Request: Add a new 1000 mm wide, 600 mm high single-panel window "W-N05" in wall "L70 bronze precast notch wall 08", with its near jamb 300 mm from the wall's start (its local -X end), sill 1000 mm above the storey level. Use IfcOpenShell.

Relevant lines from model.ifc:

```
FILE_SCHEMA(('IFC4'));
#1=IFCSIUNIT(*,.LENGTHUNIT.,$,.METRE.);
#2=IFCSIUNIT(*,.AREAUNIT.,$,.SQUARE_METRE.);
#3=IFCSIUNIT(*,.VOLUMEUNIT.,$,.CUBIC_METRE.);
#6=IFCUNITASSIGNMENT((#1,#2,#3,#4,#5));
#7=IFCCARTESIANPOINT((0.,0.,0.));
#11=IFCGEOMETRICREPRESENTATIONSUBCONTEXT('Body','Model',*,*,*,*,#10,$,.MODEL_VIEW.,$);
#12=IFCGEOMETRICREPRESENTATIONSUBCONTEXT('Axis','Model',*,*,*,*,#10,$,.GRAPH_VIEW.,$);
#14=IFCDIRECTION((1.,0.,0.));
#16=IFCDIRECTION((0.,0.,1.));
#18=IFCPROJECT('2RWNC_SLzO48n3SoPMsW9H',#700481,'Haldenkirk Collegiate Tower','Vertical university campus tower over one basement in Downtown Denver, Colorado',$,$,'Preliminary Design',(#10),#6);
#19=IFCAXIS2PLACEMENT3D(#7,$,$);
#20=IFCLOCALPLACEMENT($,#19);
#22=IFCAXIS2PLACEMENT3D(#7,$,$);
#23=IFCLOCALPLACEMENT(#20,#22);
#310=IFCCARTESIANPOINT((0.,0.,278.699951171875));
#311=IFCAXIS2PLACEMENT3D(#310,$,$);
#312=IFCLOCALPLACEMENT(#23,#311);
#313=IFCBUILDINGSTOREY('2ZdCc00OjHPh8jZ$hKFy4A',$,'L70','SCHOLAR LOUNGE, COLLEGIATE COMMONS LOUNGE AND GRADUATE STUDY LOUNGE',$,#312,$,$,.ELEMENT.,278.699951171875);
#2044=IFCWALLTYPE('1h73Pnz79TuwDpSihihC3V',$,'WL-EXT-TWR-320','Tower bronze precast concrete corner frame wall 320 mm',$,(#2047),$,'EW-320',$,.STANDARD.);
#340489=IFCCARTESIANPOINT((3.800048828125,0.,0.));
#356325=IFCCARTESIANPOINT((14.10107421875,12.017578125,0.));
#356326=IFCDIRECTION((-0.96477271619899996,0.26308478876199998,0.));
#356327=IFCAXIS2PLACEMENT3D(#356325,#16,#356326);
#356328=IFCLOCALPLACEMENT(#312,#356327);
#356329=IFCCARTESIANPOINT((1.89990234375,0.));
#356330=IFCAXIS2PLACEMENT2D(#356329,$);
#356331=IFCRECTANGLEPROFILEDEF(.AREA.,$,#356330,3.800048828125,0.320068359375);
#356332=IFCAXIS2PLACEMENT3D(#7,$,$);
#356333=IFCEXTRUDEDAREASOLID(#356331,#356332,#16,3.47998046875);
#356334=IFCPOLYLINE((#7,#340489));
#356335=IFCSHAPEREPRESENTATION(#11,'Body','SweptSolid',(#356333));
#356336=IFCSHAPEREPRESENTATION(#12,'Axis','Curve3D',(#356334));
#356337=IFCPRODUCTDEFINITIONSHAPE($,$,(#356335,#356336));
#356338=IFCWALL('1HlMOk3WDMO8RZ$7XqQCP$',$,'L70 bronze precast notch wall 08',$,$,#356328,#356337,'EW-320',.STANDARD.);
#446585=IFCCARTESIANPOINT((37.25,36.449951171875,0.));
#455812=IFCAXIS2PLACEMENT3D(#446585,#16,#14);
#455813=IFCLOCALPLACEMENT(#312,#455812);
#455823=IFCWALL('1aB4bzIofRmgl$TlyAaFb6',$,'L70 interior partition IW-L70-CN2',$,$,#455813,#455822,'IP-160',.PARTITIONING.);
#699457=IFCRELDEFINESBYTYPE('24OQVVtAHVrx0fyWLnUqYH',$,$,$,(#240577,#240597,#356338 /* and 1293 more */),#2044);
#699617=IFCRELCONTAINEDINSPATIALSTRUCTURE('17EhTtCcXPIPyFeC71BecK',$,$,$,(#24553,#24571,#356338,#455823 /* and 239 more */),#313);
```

```python
import numpy as np
import ifcopenshell
import ifcopenshell.api.feature
import ifcopenshell.api.geometry
import ifcopenshell.api.root
import ifcopenshell.api.spatial
import ifcopenshell.geom
import ifcopenshell.util.element
import ifcopenshell.util.placement
import ifcopenshell.util.representation
import ifcopenshell.util.shape
import ifcopenshell.util.unit

model = ifcopenshell.open("model.ifc")
unit_scale = ifcopenshell.util.unit.calculate_unit_scale(model)
settings = ifcopenshell.geom.settings()


def volume(element):
    """Net volume in cubic metres, openings subtracted."""
    shape = ifcopenshell.geom.create_shape(settings, element)
    return ifcopenshell.util.shape.get_volume(shape.geometry)


wall = model.by_guid("1HlMOk3WDMO8RZ$7XqQCP$")
storey = ifcopenshell.util.element.get_container(wall, ifc_class="IfcBuildingStorey")
context = ifcopenshell.util.representation.get_context(model, "Model", "Body", "MODEL_VIEW")
before = volume(wall)

width, height, from_end, sill = 1, 0.6, 0.3, 1  # metres

# The wall runs along its own X axis, and the end named is its -X end.
wall_shape = ifcopenshell.geom.create_shape(settings, wall)
x, y, z = ifcopenshell.util.shape.get_vertices(wall_shape.geometry).T
start = x.min() + from_end
face, thickness = float(y.min()), float(y.max() - y.min())
wall_matrix = ifcopenshell.util.placement.get_local_placement(wall.ObjectPlacement)
level = ifcopenshell.util.placement.get_local_placement(storey.ObjectPlacement)[2, 3]


def in_wall(x, y):
    """Placement at x, y metres in the wall's axes, at sill height."""
    matrix = wall_matrix.copy()
    matrix[:, 3] = wall_matrix @ np.array([x / unit_scale, y / unit_scale, 0.0, 1.0])
    matrix[2, 3] = level + sill / unit_scale
    return matrix


# Opening: a box that overshoots both wall faces by 50 mm.
opening = ifcopenshell.api.root.create_entity(model, ifc_class="IfcOpeningElement", predefined_type="OPENING")
box = ifcopenshell.api.geometry.add_wall_representation(
    model, context=context, length=width, height=height, thickness=thickness + 0.1
)
ifcopenshell.api.geometry.assign_representation(model, product=opening, representation=box)
ifcopenshell.api.geometry.edit_object_placement(model, product=opening, matrix=in_wall(start, face - 0.05), is_si=False)
ifcopenshell.api.feature.add_feature(model, feature=opening, element=wall)

window = ifcopenshell.api.root.create_entity(model, ifc_class="IfcWindow", name="W-N05", predefined_type="WINDOW")
window.OverallWidth, window.OverallHeight = width / unit_scale, height / unit_scale
window.PartitioningType = "SINGLE_PANEL"
body = ifcopenshell.api.geometry.add_window_representation(
    model,
    context=context,
    overall_width=window.OverallWidth,
    overall_height=window.OverallHeight,
    partition_type="SINGLE_PANEL",
)
ifcopenshell.api.geometry.assign_representation(model, product=window, representation=body)
ifcopenshell.api.spatial.assign_container(model, products=[window], relating_structure=storey)
ifcopenshell.api.feature.add_filling(model, opening=opening, element=window)

# Centre the window in the wall's thickness.
ifcopenshell.api.geometry.edit_object_placement(model, product=window, matrix=in_wall(start, face), is_si=False)
window_shape = ifcopenshell.geom.create_shape(settings, window)
depth = ifcopenshell.util.shape.get_vertices(window_shape.geometry)[:, 1]
offset = face + thickness / 2 - (depth.min() + depth.max()) / 2
ifcopenshell.api.geometry.edit_object_placement(model, product=window, matrix=in_wall(start, offset), is_si=False)

after = volume(wall)

print(f"wall volume {before:.3f} -> {after:.3f} m3")

model.write("model_v2.ifc")
```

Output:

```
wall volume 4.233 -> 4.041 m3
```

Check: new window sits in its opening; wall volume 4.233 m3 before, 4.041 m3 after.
